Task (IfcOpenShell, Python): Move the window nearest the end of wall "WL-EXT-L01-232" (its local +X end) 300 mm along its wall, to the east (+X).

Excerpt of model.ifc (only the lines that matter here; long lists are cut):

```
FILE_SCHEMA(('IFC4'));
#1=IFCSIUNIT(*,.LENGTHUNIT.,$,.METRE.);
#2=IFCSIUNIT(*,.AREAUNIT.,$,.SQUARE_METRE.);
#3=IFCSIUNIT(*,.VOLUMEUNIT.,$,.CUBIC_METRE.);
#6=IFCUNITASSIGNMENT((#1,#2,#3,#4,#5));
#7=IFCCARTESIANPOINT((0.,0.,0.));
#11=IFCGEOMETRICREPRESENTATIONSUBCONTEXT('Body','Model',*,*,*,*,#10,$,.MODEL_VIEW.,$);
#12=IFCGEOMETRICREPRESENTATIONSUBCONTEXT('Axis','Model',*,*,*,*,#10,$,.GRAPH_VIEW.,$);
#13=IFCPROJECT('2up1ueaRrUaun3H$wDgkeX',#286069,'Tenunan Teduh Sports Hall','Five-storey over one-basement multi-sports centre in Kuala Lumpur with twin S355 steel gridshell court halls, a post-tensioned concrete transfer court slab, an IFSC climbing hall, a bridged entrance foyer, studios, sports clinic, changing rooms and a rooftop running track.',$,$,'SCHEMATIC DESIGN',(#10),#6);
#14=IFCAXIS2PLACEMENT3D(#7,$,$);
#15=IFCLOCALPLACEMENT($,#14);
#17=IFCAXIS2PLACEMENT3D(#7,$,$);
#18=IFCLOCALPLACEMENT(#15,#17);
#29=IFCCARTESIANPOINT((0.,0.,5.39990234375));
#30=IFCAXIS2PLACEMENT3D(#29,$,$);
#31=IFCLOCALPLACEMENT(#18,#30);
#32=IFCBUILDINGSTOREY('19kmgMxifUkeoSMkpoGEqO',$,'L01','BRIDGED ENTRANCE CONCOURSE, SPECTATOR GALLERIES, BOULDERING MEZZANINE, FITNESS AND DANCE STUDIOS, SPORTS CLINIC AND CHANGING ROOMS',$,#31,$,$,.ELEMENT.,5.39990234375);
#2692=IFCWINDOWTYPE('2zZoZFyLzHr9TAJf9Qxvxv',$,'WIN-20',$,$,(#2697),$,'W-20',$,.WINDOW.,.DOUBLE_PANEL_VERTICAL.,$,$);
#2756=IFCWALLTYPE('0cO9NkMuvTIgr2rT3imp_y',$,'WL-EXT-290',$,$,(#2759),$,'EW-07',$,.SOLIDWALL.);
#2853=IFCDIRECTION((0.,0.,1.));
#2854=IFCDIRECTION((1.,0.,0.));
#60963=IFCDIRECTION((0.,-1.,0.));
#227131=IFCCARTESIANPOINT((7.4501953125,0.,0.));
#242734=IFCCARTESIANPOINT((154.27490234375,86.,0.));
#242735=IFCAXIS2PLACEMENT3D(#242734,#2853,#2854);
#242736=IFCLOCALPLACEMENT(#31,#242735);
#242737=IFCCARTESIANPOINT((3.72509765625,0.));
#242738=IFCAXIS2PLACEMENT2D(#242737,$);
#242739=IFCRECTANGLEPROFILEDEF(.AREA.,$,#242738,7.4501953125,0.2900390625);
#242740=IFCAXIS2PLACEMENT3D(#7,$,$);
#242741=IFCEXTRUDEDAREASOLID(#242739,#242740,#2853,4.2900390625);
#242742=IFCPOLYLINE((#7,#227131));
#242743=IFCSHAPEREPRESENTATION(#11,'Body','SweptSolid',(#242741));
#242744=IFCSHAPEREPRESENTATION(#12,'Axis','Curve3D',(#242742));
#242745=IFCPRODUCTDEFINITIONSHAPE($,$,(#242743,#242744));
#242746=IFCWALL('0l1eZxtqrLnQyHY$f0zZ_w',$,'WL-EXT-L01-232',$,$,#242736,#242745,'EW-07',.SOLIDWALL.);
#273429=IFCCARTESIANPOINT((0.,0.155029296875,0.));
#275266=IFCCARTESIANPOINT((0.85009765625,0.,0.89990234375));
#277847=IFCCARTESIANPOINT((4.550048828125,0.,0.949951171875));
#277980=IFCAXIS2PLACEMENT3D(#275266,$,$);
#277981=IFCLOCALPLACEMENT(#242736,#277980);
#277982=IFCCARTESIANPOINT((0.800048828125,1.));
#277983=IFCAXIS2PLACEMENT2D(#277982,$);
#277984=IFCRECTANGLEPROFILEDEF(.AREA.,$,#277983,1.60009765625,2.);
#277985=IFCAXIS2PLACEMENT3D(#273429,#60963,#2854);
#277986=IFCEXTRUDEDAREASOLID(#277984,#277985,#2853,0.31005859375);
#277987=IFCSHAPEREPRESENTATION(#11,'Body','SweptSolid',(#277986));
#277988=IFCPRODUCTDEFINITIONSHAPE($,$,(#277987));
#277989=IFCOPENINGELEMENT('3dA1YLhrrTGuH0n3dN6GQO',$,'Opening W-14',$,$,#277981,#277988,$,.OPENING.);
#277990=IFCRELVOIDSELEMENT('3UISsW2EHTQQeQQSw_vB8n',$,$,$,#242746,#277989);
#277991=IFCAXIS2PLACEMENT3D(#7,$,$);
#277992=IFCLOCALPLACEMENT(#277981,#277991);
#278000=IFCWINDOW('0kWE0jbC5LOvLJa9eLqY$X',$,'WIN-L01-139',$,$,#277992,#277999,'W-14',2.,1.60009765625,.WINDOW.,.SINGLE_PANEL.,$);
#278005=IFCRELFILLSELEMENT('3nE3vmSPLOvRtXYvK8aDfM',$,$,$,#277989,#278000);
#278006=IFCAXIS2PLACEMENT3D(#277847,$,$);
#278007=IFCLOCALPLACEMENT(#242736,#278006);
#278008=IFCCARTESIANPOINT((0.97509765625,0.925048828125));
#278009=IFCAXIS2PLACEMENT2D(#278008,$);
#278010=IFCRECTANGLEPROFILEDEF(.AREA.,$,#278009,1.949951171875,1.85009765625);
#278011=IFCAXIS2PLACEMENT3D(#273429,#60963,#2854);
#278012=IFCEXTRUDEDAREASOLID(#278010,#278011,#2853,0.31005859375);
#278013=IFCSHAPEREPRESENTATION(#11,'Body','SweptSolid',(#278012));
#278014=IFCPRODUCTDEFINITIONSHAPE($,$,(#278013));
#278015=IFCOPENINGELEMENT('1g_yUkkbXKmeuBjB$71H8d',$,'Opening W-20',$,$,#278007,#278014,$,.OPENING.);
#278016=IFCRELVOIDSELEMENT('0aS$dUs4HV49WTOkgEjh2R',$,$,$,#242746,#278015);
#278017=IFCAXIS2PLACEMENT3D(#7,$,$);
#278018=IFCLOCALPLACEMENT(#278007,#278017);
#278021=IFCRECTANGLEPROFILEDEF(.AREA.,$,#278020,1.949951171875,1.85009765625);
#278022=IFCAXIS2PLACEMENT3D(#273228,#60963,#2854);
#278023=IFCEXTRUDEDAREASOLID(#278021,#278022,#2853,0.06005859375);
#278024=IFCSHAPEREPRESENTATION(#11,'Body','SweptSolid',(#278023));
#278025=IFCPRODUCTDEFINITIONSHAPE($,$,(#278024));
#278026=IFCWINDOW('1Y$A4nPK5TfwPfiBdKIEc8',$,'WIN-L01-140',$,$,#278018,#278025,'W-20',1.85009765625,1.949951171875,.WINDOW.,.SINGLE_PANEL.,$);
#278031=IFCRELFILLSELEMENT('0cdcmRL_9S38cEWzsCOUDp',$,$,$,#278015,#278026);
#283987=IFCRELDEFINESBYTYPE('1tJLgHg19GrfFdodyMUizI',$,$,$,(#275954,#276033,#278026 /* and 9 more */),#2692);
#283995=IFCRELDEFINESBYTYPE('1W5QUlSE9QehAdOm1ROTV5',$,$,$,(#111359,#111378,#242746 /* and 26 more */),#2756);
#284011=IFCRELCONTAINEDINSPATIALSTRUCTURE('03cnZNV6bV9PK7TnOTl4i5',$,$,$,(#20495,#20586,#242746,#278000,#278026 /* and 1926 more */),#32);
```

```python
import ifcopenshell
import ifcopenshell.api.geometry
import ifcopenshell.util.placement

model = ifcopenshell.open("model.ifc")

window = model.by_guid("1Y$A4nPK5TfwPfiBdKIEc8")
opening = window.FillsVoids[0].RelatingOpeningElement
wall = opening.VoidsElements[0].RelatingBuildingElement

wall_matrix = ifcopenshell.util.placement.get_local_placement(wall.ObjectPlacement)
shift = wall_matrix[:3, 0] * 0.3
before = ifcopenshell.util.placement.get_local_placement(window.ObjectPlacement)[:3, 3].copy()

# The window is placed relative to its opening, so it follows when the opening moves.
matrix = ifcopenshell.util.placement.get_local_placement(opening.ObjectPlacement)
matrix[:3, 3] += shift
ifcopenshell.api.geometry.edit_object_placement(
    model, product=opening, matrix=matrix, is_si=False, should_transform_children=True
)

after = ifcopenshell.util.placement.get_local_placement(window.ObjectPlacement)[:3, 3]
print("window moved by", (after - before).round(3) + 0.0)

model.write("model_v2.ifc")
```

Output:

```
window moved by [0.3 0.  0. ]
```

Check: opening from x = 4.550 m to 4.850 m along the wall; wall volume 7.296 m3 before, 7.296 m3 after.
